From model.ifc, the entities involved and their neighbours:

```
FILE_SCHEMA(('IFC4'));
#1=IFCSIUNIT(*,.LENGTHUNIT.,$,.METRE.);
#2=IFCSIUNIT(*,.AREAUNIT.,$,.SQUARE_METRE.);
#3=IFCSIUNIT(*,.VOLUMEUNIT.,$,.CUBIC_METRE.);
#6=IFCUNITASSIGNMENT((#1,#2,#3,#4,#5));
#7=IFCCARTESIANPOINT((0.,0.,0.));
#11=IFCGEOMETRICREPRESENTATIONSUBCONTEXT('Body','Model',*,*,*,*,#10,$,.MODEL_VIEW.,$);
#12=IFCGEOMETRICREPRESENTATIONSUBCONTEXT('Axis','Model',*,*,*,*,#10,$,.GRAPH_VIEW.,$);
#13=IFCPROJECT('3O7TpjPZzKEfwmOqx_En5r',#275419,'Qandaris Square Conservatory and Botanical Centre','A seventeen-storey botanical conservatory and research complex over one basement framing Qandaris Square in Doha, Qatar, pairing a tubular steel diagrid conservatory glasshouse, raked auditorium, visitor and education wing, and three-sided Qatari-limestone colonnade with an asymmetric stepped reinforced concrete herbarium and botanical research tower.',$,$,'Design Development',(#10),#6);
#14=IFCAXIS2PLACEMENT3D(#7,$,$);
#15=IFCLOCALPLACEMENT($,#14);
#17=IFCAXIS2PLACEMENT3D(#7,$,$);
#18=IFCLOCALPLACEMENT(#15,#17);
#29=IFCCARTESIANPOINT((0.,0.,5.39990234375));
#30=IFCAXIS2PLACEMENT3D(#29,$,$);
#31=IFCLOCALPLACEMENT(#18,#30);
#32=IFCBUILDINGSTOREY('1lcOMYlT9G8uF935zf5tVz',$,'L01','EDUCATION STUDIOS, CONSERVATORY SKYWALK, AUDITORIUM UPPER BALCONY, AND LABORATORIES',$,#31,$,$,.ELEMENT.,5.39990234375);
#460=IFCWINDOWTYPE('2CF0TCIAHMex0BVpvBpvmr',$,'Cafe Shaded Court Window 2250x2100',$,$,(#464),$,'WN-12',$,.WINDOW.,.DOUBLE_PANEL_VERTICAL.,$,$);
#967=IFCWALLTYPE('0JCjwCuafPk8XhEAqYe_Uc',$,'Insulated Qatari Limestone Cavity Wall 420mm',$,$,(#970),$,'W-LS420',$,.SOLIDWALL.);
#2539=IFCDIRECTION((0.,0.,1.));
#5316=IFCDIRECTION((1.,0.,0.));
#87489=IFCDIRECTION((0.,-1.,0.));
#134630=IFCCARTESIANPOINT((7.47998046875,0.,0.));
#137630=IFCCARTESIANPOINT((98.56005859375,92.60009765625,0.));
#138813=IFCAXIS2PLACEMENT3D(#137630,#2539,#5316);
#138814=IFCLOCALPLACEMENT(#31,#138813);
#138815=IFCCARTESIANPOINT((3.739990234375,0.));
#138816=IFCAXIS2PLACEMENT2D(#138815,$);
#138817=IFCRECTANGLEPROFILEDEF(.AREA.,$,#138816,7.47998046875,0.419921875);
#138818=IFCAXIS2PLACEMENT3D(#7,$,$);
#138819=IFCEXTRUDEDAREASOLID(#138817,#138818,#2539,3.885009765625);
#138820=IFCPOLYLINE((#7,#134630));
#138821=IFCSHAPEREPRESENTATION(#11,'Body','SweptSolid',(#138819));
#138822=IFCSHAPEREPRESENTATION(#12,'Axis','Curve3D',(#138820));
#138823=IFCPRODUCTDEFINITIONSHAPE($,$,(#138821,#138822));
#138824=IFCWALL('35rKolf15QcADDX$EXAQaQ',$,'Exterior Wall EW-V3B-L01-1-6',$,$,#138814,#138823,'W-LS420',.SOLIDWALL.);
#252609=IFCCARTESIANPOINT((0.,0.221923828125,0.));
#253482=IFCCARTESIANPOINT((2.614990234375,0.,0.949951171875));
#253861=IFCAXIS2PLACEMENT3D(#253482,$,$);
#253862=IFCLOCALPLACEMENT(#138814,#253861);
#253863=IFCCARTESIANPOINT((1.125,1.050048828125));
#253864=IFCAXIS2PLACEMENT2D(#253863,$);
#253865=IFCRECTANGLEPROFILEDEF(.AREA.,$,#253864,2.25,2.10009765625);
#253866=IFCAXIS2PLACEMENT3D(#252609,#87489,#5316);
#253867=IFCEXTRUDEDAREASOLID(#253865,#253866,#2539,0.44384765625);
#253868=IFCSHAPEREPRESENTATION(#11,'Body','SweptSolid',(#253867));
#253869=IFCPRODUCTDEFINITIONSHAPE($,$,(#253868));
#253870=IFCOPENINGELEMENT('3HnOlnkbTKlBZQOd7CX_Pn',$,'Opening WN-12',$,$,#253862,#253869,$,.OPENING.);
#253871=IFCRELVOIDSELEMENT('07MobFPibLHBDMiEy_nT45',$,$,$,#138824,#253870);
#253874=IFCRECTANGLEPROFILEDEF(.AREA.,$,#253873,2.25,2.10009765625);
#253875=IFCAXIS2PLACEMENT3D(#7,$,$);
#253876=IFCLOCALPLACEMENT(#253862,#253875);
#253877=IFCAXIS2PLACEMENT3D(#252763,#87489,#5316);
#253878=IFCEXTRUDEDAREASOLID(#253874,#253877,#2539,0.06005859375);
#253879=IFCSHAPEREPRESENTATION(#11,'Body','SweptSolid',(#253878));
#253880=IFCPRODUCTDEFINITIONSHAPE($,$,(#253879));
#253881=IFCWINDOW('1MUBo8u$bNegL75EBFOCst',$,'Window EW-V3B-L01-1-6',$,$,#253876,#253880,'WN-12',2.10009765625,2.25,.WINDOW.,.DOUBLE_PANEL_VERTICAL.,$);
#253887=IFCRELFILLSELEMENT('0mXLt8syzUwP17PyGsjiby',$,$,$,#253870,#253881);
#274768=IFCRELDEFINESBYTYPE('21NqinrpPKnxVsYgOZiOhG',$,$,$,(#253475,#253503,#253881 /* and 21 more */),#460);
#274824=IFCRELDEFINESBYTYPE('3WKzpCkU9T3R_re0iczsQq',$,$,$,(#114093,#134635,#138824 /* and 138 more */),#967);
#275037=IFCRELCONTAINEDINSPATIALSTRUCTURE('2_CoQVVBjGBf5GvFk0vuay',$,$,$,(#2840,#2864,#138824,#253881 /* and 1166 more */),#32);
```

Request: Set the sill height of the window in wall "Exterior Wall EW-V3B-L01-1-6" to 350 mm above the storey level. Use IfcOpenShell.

```python
import numpy as np
import ifcopenshell
import ifcopenshell.api.geometry
import ifcopenshell.geom
import ifcopenshell.util.element
import ifcopenshell.util.placement
import ifcopenshell.util.shape
import ifcopenshell.util.unit

model = ifcopenshell.open("model.ifc")
unit_scale = ifcopenshell.util.unit.calculate_unit_scale(model)

window = model.by_guid("1MUBo8u$bNegL75EBFOCst")
opening = window.FillsVoids[0].RelatingOpeningElement
storey = ifcopenshell.util.element.get_container(window, ifc_class="IfcBuildingStorey")
level = ifcopenshell.util.placement.get_local_placement(storey.ObjectPlacement)[2, 3]

# The opening's origin need not be at the sill, so measure its lowest point.
shape = ifcopenshell.geom.create_shape(ifcopenshell.geom.settings(), opening)
bottom = ifcopenshell.util.shape.get_shape_bottom_elevation(shape, shape.geometry) / unit_scale
dz = level + 0.35 - bottom

shift = np.array([0.0, 0.0, dz])
# The window is placed relative to its opening, so it follows when the opening moves.
matrix = ifcopenshell.util.placement.get_local_placement(opening.ObjectPlacement)
matrix[:3, 3] += shift
ifcopenshell.api.geometry.edit_object_placement(
    model, product=opening, matrix=matrix, is_si=False, should_transform_children=True
)

print(f"moved by {dz * unit_scale:+.3f} m")

model.write("model_v2.ifc")
```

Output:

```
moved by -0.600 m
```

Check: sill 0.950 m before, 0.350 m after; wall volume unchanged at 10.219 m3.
